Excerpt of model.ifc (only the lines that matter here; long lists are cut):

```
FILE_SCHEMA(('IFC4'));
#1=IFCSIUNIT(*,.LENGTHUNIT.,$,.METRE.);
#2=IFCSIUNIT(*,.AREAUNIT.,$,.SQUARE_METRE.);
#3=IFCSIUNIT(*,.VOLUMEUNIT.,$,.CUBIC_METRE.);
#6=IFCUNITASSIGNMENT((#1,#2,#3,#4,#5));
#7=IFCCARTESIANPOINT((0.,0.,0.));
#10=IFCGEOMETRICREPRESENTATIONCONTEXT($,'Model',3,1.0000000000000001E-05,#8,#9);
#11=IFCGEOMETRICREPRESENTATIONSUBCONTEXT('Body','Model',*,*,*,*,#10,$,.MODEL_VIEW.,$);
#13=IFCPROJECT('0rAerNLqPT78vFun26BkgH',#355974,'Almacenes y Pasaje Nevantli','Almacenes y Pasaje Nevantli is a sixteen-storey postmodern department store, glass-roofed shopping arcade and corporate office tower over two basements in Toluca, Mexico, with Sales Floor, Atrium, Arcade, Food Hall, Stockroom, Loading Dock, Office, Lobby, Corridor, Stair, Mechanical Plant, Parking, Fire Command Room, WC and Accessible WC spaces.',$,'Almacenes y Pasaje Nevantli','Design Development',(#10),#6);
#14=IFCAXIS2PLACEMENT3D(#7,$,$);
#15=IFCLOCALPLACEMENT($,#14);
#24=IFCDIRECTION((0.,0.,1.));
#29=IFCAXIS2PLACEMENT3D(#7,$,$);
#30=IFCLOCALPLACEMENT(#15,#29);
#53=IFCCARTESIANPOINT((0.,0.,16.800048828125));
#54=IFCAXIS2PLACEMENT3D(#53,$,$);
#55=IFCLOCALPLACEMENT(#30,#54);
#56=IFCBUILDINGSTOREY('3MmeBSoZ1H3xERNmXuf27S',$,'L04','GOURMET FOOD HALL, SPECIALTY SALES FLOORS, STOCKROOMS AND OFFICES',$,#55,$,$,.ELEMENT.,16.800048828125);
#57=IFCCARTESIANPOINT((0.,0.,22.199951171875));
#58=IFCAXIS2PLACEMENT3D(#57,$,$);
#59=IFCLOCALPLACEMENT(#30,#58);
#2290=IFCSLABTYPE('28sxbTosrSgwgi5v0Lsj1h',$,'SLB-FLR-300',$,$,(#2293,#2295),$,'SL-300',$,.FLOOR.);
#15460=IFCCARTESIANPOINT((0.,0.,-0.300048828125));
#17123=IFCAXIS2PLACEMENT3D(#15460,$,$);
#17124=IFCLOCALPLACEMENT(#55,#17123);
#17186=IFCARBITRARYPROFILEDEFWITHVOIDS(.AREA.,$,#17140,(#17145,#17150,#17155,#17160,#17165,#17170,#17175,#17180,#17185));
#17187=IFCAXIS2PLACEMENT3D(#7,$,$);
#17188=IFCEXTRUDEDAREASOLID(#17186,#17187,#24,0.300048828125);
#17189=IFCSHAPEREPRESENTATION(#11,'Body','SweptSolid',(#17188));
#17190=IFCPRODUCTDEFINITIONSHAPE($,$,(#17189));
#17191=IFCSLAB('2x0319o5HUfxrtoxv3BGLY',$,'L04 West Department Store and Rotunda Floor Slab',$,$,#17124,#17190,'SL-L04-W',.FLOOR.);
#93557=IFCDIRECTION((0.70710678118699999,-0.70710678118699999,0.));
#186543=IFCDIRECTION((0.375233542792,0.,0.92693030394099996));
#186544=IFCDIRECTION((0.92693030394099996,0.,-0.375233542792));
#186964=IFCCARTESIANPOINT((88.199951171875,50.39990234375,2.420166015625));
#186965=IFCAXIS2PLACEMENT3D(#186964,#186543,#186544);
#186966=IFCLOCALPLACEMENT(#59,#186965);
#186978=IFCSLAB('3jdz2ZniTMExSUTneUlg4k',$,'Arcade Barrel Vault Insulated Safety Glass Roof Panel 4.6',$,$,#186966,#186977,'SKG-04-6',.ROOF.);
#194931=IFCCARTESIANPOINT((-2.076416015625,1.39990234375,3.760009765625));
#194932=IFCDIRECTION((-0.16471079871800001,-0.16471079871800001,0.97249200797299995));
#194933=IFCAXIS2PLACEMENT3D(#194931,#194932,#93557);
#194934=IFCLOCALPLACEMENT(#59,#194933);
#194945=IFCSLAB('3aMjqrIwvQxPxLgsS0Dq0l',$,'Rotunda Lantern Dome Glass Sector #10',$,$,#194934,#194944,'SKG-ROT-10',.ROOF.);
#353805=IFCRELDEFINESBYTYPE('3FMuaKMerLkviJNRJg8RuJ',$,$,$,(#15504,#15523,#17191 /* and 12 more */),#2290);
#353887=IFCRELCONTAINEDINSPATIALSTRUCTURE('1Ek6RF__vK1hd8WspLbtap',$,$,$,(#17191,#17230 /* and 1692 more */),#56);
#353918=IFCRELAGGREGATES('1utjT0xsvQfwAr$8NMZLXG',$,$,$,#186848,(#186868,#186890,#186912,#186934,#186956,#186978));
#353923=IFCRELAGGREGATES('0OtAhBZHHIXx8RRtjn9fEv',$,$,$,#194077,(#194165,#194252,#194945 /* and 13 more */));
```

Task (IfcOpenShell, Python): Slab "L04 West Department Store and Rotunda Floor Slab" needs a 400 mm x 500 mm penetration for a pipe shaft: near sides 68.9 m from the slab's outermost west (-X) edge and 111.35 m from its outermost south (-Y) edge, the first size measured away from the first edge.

```python
import numpy as np
import ifcopenshell
import ifcopenshell.api.feature
import ifcopenshell.api.geometry
import ifcopenshell.api.root
import ifcopenshell.geom
import ifcopenshell.util.placement
import ifcopenshell.util.representation
import ifcopenshell.util.shape
import ifcopenshell.util.unit

model = ifcopenshell.open("model.ifc")
unit_scale = ifcopenshell.util.unit.calculate_unit_scale(model)
settings = ifcopenshell.geom.settings()


def volume(element):
    """Net volume in cubic metres, openings subtracted."""
    shape = ifcopenshell.geom.create_shape(settings, element)
    return ifcopenshell.util.shape.get_volume(shape.geometry)


slab = model.by_guid("2x0319o5HUfxrtoxv3BGLY")
before = volume(slab)

# Extent in the slab's own axes, in metres. The edges named are its -X and -Y sides.
slab_shape = ifcopenshell.geom.create_shape(settings, slab)
vertices = ifcopenshell.util.shape.get_vertices(slab_shape.geometry)
x_min, y_min, bottom = vertices.min(axis=0)
top = vertices[:, 2].max()

opening = ifcopenshell.api.root.create_entity(model, ifc_class="IfcOpeningElement", name="Pipe shaft opening", predefined_type="OPENING")
context = ifcopenshell.util.representation.get_context(model, "Model", "Body", "MODEL_VIEW")
width, depth = 0.4, 0.5
outline = [(0.0, 0.0), (width, 0.0), (width, depth), (0.0, depth), (0.0, 0.0)]
# Overshoot both faces by 50 mm so the cut is clean.
shape = ifcopenshell.api.geometry.add_slab_representation(
    model, context=context, depth=top - bottom + 0.1, polyline=outline
)
ifcopenshell.api.geometry.assign_representation(model, product=opening, representation=shape)

matrix = ifcopenshell.util.placement.get_local_placement(slab.ObjectPlacement)
matrix[:, 3] = matrix @ np.append(np.array([x_min + 68.9, y_min + 111.35, bottom - 0.05]) / unit_scale, 1.0)
ifcopenshell.api.geometry.edit_object_placement(model, product=opening, matrix=matrix, is_si=False)
ifcopenshell.api.feature.add_feature(model, feature=opening, element=slab)

after = volume(slab)

print(f"slab volume {before:.3f} -> {after:.3f} m3")

model.write("model_rev.ifc")
```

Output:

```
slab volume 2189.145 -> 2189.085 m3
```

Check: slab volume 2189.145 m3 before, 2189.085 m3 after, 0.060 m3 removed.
